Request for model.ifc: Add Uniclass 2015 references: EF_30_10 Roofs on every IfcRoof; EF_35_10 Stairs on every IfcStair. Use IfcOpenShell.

First a look at what the model holds.

```python
import ifcopenshell

model = ifcopenshell.open("model.ifc")
print(model.schema)
print("classifications:", [c.Name for c in model.by_type("IfcClassification")])
for ifc_class in ("IfcDoor", "IfcRoof", "IfcStair", "IfcWall", "IfcWindow"):
    print(ifc_class, len(model.by_type(ifc_class)))
```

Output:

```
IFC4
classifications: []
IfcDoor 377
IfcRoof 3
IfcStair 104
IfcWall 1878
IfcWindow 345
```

```python
import ifcopenshell
import ifcopenshell.api.classification

model = ifcopenshell.open("model.ifc")

system = ifcopenshell.api.classification.add_classification(model, classification="Uniclass 2015")

codes = {
    "IfcRoof": ("EF_30_10", "Roofs"),
    "IfcStair": ("EF_35_10", "Stairs"),
}
for ifc_class, (code, name) in codes.items():
    products = model.by_type(ifc_class)
    ifcopenshell.api.classification.add_reference(
        model, products=products, classification=system, identification=code, name=name
    )
    print(code, len(products))

model.write("model_v2.ifc")
```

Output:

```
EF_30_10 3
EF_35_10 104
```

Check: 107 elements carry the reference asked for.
